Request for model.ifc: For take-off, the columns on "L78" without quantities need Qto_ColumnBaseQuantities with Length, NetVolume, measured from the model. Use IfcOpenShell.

First a look at what the model holds.

```python
import ifcopenshell
import ifcopenshell.util.element
import ifcopenshell.util.unit

model = ifcopenshell.open("model.ifc")
print(model.schema)
for unit_type in ("LENGTHUNIT", "AREAUNIT", "VOLUMEUNIT"):
    print(unit_type, ifcopenshell.util.unit.calculate_unit_scale(model, unit_type))
storey = next(s for s in model.by_type("IfcBuildingStorey") if s.Name == "L78")
columns = [e for e in ifcopenshell.util.element.get_decomposition(storey) if e.is_a("IfcColumn")]
for e in sorted(columns, key=lambda e: e.id()):
    print(e.id(), e.is_a(), e.Name, list(ifcopenshell.util.element.get_psets(e, qtos_only=True)), sep=" | ")
```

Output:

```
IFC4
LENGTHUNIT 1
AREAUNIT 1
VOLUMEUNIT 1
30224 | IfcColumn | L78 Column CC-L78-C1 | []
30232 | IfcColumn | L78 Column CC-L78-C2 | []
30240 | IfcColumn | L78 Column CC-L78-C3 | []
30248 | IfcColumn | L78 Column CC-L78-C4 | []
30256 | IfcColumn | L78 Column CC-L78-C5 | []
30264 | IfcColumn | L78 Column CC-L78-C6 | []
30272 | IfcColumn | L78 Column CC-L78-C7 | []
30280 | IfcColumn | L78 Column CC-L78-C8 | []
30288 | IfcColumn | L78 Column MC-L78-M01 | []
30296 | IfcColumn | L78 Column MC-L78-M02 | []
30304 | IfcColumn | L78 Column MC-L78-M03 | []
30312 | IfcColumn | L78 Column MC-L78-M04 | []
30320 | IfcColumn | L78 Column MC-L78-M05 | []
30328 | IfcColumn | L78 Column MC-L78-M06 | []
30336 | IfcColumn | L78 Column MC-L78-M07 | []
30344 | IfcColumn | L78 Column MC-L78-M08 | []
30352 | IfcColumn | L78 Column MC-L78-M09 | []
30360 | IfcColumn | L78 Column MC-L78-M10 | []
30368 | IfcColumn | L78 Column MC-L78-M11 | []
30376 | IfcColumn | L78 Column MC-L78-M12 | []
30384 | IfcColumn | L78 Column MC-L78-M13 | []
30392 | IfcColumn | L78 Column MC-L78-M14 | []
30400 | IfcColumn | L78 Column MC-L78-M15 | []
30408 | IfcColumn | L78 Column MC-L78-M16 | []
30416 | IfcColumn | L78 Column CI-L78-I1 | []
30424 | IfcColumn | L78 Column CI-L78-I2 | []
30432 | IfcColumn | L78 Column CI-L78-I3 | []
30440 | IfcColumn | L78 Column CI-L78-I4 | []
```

```python
import ifcopenshell
import ifcopenshell.api.pset
import ifcopenshell.geom
import ifcopenshell.util.element
import ifcopenshell.util.shape
import ifcopenshell.util.unit

model = ifcopenshell.open("model.ifc")
unit_scale = ifcopenshell.util.unit.calculate_unit_scale(model)
volume_scale = ifcopenshell.util.unit.calculate_unit_scale(model, "VOLUMEUNIT")
settings = ifcopenshell.geom.settings()

storey = next(s for s in model.by_type("IfcBuildingStorey") if s.Name == "L78")
columns = [e for e in ifcopenshell.util.element.get_decomposition(storey) if e.is_a("IfcColumn")]

for e in sorted(columns, key=lambda e: e.id()):
    if ifcopenshell.util.element.get_psets(e, qtos_only=True, should_inherit=False):
        continue
    # Geometry comes back in metres, in the element's own axes.
    shape = ifcopenshell.geom.create_shape(settings, e)
    values = {
        "Length": ifcopenshell.util.shape.get_z(shape.geometry) / unit_scale,
        "NetVolume": ifcopenshell.util.shape.get_volume(shape.geometry) / volume_scale,
    }
    qto = ifcopenshell.api.pset.add_qto(model, product=e, name="Qto_ColumnBaseQuantities")
    ifcopenshell.api.pset.edit_qto(model, qto=qto, properties=values)
    print(e.id(), {k: round(v, 3) for k, v in values.items()})

model.write("model_v2.ifc")
```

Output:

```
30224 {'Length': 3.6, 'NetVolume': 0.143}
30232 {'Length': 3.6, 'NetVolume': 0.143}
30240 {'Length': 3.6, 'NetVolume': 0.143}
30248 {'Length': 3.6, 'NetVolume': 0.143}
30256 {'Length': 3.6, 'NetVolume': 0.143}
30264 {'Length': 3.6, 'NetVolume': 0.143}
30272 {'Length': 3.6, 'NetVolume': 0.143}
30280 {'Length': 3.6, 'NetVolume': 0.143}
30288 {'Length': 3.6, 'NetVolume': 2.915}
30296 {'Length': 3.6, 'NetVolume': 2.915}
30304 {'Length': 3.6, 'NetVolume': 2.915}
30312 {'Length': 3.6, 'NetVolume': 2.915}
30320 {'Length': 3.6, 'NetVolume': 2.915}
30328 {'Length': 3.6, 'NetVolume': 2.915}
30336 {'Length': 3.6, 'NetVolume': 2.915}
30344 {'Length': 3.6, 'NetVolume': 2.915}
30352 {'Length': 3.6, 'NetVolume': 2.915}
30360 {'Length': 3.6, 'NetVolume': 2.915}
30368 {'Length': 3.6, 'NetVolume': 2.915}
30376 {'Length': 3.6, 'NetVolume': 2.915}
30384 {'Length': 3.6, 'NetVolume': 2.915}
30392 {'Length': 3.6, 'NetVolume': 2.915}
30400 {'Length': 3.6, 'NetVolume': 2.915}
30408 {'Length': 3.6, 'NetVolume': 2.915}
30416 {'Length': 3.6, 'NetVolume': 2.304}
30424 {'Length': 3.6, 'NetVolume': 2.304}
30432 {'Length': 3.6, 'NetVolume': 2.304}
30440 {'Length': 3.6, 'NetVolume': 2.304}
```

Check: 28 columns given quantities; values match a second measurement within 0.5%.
